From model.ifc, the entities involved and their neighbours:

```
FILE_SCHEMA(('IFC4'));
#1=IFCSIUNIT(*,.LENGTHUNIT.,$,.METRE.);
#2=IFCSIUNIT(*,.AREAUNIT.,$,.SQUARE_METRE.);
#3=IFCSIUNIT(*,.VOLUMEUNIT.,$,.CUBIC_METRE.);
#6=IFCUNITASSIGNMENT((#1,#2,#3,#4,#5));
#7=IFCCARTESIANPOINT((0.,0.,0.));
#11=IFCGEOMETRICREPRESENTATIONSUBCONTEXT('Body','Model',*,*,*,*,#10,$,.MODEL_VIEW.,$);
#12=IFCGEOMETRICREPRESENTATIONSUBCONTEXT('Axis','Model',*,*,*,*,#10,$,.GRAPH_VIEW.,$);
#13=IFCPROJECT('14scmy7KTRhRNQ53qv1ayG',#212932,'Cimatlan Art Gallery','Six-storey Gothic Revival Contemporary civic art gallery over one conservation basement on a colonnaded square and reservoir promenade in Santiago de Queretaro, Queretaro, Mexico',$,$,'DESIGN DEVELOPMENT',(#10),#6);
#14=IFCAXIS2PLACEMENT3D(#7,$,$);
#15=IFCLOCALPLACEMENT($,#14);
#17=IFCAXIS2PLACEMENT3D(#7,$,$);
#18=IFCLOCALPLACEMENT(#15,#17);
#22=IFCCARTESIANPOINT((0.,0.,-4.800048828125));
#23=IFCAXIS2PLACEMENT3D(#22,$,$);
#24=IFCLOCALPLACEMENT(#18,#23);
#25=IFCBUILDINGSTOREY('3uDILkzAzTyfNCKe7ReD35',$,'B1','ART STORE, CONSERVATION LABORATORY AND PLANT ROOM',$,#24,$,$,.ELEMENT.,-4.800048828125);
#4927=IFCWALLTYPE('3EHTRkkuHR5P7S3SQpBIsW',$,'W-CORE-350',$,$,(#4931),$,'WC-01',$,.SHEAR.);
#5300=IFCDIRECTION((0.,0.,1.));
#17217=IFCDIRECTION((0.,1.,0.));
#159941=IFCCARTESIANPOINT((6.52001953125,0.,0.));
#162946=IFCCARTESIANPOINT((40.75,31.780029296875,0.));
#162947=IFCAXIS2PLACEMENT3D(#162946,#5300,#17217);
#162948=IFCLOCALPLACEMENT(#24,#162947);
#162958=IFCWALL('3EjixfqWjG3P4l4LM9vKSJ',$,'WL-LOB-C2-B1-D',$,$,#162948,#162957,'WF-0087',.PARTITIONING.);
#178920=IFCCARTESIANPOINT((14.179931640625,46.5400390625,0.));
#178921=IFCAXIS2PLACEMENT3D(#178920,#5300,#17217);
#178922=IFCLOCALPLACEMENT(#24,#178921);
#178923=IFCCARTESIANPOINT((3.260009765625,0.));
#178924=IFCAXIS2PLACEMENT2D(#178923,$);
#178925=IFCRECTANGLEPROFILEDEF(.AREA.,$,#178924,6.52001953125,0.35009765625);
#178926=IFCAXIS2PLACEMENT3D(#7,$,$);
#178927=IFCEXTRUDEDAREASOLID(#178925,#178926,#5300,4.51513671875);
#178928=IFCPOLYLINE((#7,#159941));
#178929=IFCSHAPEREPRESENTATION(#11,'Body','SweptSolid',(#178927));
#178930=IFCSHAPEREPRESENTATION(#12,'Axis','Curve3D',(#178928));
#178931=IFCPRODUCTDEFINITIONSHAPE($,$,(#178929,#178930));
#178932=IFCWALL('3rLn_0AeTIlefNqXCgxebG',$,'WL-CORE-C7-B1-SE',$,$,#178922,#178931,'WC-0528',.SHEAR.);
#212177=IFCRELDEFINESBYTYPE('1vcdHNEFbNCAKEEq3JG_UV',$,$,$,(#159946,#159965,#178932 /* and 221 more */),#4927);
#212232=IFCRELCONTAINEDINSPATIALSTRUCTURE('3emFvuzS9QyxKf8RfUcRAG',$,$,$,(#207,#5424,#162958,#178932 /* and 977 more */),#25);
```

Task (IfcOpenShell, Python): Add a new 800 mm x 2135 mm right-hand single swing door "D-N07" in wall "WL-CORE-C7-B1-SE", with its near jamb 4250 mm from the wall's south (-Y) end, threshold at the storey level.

```python
import numpy as np
import ifcopenshell
import ifcopenshell.api.feature
import ifcopenshell.api.geometry
import ifcopenshell.api.root
import ifcopenshell.api.spatial
import ifcopenshell.geom
import ifcopenshell.util.element
import ifcopenshell.util.placement
import ifcopenshell.util.representation
import ifcopenshell.util.shape
import ifcopenshell.util.unit

model = ifcopenshell.open("model.ifc")
unit_scale = ifcopenshell.util.unit.calculate_unit_scale(model)
settings = ifcopenshell.geom.settings()


def volume(element):
    """Net volume in cubic metres, openings subtracted."""
    shape = ifcopenshell.geom.create_shape(settings, element)
    return ifcopenshell.util.shape.get_volume(shape.geometry)


wall = model.by_id(178932)
storey = ifcopenshell.util.element.get_container(wall, ifc_class="IfcBuildingStorey")
context = ifcopenshell.util.representation.get_context(model, "Model", "Body", "MODEL_VIEW")
before = volume(wall)

width, height, from_end, sill = 0.8, 2.135, 4.25, 0.0  # metres

# The wall runs along its own X axis, and the end named is its -X end.
wall_shape = ifcopenshell.geom.create_shape(settings, wall)
x, y, z = ifcopenshell.util.shape.get_vertices(wall_shape.geometry).T
start = x.min() + from_end
face, thickness = float(y.min()), float(y.max() - y.min())
wall_matrix = ifcopenshell.util.placement.get_local_placement(wall.ObjectPlacement)
level = ifcopenshell.util.placement.get_local_placement(storey.ObjectPlacement)[2, 3]


def in_wall(x, y):
    """Placement at x, y metres in the wall's axes, at sill height."""
    matrix = wall_matrix.copy()
    matrix[:, 3] = wall_matrix @ np.array([x / unit_scale, y / unit_scale, 0.0, 1.0])
    matrix[2, 3] = level + sill / unit_scale
    return matrix


# Opening: a box that overshoots both wall faces by 50 mm.
opening = ifcopenshell.api.root.create_entity(model, ifc_class="IfcOpeningElement", predefined_type="OPENING")
box = ifcopenshell.api.geometry.add_wall_representation(
    model, context=context, length=width, height=height, thickness=thickness + 0.1
)
ifcopenshell.api.geometry.assign_representation(model, product=opening, representation=box)
ifcopenshell.api.geometry.edit_object_placement(model, product=opening, matrix=in_wall(start, face - 0.05), is_si=False)
ifcopenshell.api.feature.add_feature(model, feature=opening, element=wall)

door = ifcopenshell.api.root.create_entity(model, ifc_class="IfcDoor", name="D-N07", predefined_type="DOOR")
door.OverallWidth, door.OverallHeight = width / unit_scale, height / unit_scale
door.OperationType = "SINGLE_SWING_RIGHT"
body = ifcopenshell.api.geometry.add_door_representation(
    model,
    context=context,
    overall_width=door.OverallWidth,
    overall_height=door.OverallHeight,
    operation_type="SINGLE_SWING_RIGHT",
    lining_properties={"LiningDepth": thickness / unit_scale, "ThresholdDepth": thickness / unit_scale},
)
ifcopenshell.api.geometry.assign_representation(model, product=door, representation=body)
ifcopenshell.api.spatial.assign_container(model, products=[door], relating_structure=storey)
ifcopenshell.api.feature.add_filling(model, opening=opening, element=door)

# The lining spans the wall, so the door starts at the wall face.
ifcopenshell.api.geometry.edit_object_placement(model, product=door, matrix=in_wall(start, face), is_si=False)

after = volume(wall)

print(f"wall volume {before:.3f} -> {after:.3f} m3")

model.write("model_v2.ifc")
```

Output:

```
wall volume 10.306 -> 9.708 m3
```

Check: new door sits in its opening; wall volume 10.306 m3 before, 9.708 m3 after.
